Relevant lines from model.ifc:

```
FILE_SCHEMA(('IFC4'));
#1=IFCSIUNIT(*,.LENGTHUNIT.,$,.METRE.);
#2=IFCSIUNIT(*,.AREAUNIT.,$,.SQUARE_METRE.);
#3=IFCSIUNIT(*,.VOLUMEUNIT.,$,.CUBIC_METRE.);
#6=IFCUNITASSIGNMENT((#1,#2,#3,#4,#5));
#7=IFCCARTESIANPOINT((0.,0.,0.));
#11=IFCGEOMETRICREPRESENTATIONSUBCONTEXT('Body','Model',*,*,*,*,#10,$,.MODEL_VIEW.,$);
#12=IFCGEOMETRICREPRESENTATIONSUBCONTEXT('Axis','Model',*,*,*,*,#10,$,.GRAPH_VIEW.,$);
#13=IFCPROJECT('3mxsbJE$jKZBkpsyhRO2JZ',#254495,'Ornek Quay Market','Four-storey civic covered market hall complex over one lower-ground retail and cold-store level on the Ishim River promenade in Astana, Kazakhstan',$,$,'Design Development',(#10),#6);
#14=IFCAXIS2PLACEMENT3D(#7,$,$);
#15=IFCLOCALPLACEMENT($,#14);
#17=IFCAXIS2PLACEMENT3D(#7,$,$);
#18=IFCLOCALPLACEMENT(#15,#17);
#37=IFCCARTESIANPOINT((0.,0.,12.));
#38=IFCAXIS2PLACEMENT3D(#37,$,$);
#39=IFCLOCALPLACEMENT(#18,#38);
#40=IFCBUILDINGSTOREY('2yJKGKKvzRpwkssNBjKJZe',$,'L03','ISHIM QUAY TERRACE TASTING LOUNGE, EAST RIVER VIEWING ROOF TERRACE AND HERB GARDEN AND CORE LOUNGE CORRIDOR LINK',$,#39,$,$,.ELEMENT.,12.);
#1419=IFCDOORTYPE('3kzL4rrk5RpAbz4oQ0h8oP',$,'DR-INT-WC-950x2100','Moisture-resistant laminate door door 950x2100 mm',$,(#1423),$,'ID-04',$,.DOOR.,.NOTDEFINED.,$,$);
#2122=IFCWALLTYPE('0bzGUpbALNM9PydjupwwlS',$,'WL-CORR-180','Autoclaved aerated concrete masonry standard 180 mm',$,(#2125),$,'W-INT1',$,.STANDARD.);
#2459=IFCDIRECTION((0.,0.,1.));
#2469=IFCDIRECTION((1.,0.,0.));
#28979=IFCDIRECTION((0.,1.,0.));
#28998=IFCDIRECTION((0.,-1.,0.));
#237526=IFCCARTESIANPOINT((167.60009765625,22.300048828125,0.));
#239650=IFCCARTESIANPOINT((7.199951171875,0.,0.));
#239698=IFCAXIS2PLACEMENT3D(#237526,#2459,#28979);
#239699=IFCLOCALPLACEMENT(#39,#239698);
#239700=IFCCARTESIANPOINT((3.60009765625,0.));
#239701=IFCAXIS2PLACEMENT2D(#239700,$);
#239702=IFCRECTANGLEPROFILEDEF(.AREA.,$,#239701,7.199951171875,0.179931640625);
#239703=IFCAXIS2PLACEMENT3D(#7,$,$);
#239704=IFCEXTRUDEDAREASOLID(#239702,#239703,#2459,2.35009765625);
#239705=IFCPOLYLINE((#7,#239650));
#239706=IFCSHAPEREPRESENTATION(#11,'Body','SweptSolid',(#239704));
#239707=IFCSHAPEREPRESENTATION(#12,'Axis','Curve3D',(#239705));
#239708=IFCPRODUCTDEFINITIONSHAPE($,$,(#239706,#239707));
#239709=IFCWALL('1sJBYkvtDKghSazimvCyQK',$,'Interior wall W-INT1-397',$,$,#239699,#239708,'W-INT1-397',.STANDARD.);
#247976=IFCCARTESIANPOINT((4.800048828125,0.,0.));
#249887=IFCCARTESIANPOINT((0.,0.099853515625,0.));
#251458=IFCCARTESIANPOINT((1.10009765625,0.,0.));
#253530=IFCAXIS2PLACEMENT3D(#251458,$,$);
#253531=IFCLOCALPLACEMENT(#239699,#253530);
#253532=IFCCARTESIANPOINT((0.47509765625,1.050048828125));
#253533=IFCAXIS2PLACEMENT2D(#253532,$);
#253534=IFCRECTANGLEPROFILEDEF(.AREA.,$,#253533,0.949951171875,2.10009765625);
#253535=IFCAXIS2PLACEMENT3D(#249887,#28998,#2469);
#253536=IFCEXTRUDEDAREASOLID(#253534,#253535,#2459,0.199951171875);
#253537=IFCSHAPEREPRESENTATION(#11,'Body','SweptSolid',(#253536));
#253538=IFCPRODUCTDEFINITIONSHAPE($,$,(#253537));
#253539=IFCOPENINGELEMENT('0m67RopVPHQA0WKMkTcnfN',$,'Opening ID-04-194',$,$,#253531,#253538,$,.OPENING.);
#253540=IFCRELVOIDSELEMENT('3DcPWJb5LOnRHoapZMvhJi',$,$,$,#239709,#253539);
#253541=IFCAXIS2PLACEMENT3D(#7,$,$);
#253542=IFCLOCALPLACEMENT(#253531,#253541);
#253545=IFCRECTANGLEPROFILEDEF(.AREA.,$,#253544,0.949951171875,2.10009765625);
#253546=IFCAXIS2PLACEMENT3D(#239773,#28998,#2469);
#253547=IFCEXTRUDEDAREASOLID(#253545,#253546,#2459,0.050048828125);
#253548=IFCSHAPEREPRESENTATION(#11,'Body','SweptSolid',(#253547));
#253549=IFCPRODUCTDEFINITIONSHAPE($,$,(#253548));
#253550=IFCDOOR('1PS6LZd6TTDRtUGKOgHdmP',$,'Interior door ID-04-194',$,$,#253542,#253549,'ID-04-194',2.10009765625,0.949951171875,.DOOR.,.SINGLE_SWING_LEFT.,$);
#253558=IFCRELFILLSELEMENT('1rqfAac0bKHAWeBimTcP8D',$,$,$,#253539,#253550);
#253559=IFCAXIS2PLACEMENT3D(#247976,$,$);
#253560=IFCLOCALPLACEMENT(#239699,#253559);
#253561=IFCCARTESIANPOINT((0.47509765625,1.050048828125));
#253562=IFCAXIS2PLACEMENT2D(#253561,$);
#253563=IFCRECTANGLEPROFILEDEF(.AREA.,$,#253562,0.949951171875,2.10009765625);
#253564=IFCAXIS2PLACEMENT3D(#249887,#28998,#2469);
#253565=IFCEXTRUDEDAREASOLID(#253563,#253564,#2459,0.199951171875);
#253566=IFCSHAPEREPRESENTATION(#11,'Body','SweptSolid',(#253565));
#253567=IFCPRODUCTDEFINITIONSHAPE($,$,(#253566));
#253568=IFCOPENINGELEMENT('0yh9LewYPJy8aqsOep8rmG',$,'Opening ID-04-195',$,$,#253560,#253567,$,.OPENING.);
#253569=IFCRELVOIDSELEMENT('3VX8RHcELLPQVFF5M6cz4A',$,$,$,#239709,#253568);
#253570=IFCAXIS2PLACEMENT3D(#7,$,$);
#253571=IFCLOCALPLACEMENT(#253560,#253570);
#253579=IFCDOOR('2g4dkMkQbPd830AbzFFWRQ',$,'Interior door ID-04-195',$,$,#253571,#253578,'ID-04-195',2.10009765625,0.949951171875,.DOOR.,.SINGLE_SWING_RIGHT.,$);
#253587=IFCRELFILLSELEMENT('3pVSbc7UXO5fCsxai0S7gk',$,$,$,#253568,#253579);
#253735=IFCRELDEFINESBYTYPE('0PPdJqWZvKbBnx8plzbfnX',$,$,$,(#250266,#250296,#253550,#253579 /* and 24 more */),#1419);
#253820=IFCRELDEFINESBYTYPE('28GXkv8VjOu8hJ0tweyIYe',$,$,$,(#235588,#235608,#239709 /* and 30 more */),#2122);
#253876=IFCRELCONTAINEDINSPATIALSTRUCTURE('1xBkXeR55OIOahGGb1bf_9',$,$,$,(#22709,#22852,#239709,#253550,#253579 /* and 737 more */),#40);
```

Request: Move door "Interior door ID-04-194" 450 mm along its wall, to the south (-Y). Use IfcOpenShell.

```python
import ifcopenshell
import ifcopenshell.api.geometry
import ifcopenshell.util.placement
import ifcopenshell.util.unit

model = ifcopenshell.open("model.ifc")
unit_scale = ifcopenshell.util.unit.calculate_unit_scale(model)

door = model.by_id(253550)
opening = door.FillsVoids[0].RelatingOpeningElement
wall = opening.VoidsElements[0].RelatingBuildingElement

wall_matrix = ifcopenshell.util.placement.get_local_placement(wall.ObjectPlacement)
shift = wall_matrix[:3, 0] * -0.45 / unit_scale
before = ifcopenshell.util.placement.get_local_placement(door.ObjectPlacement)[:3, 3].copy()

# The door is placed relative to its opening, so it follows when the opening moves.
matrix = ifcopenshell.util.placement.get_local_placement(opening.ObjectPlacement)
matrix[:3, 3] += shift
ifcopenshell.api.geometry.edit_object_placement(
    model, product=opening, matrix=matrix, is_si=False, should_transform_children=True
)

after = ifcopenshell.util.placement.get_local_placement(door.ObjectPlacement)[:3, 3]
print("door moved by", (after - before).round(3) + 0.0)

model.write("model_updated.ifc")
```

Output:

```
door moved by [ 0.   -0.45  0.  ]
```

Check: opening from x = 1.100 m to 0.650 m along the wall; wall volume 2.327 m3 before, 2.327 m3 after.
